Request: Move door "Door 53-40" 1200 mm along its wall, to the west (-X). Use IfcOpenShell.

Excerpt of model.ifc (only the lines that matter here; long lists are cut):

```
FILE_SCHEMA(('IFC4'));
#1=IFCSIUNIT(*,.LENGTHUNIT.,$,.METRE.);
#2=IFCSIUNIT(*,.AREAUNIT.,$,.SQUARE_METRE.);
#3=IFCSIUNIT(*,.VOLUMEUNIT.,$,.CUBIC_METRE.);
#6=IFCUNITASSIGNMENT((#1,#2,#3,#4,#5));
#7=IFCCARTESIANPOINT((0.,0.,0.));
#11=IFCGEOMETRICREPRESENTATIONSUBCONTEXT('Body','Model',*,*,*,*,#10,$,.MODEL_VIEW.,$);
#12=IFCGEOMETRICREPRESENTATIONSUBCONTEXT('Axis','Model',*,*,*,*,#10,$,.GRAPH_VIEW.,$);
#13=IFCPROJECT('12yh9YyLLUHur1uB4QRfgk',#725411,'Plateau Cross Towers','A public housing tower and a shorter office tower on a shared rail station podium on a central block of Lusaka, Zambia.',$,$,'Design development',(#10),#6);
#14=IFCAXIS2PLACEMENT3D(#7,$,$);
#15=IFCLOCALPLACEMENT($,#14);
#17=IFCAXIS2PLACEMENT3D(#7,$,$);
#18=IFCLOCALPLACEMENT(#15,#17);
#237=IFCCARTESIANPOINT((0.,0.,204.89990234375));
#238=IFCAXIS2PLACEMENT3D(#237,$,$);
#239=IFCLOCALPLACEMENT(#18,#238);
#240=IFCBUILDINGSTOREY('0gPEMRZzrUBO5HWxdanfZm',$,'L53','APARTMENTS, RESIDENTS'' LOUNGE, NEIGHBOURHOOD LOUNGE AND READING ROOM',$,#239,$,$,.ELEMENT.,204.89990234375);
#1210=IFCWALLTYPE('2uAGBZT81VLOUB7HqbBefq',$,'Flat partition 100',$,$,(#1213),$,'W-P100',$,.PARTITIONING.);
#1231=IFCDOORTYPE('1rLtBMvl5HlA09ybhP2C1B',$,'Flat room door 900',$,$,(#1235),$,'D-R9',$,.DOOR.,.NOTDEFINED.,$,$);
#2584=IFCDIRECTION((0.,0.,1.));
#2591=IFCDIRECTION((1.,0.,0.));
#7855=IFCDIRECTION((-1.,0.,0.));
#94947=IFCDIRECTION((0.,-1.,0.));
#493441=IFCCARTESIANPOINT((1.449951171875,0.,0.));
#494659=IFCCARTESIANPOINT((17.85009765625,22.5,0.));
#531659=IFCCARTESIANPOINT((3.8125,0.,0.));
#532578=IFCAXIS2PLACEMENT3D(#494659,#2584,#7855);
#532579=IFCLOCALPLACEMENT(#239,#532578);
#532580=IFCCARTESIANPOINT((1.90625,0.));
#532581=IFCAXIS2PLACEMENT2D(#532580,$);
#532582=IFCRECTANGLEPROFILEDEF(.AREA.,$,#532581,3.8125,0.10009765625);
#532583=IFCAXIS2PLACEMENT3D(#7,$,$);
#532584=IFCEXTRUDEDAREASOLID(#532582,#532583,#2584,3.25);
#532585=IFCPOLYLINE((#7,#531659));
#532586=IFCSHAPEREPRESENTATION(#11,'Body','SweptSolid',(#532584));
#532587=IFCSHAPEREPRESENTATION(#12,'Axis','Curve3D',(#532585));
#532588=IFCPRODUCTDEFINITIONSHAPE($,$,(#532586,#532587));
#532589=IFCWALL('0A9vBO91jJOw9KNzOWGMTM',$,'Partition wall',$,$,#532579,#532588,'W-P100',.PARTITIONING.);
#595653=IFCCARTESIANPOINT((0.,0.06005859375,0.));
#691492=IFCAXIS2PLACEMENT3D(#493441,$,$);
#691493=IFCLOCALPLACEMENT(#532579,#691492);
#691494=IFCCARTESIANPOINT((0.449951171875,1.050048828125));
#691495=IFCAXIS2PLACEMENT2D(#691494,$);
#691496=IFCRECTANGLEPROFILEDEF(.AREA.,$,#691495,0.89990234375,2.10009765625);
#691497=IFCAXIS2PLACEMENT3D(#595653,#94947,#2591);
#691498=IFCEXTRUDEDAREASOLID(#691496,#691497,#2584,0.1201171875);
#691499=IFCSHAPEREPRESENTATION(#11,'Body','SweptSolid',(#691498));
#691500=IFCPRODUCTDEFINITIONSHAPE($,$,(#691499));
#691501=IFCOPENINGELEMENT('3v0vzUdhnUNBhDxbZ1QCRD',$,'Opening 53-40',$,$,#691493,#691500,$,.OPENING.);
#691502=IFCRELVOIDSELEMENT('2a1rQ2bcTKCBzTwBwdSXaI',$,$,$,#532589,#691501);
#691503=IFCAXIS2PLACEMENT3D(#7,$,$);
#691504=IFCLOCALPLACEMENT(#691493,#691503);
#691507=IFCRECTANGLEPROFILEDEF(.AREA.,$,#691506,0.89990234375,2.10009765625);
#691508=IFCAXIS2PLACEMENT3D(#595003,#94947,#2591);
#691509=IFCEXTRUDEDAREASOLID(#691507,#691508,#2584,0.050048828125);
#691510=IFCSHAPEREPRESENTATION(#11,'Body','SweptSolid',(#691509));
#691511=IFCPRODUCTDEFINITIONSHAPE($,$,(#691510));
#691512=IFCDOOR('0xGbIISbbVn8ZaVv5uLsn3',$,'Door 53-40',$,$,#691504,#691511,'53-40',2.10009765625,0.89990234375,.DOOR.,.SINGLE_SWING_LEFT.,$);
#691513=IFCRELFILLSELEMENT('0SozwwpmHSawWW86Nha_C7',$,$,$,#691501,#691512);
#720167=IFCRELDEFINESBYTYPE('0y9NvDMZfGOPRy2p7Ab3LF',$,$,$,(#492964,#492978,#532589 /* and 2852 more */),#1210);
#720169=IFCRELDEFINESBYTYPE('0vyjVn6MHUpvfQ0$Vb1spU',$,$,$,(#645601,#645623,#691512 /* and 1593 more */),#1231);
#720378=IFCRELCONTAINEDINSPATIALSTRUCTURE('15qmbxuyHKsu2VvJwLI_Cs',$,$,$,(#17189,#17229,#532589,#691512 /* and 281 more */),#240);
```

```python
import ifcopenshell
import ifcopenshell.api.geometry
import ifcopenshell.util.placement
import ifcopenshell.util.unit

model = ifcopenshell.open("model.ifc")
unit_scale = ifcopenshell.util.unit.calculate_unit_scale(model)

door = model.by_guid("0xGbIISbbVn8ZaVv5uLsn3")
opening = door.FillsVoids[0].RelatingOpeningElement
wall = opening.VoidsElements[0].RelatingBuildingElement

wall_matrix = ifcopenshell.util.placement.get_local_placement(wall.ObjectPlacement)
shift = wall_matrix[:3, 0] * 1.2 / unit_scale
before = ifcopenshell.util.placement.get_local_placement(door.ObjectPlacement)[:3, 3].copy()

# The door is placed relative to its opening, so it follows when the opening moves.
matrix = ifcopenshell.util.placement.get_local_placement(opening.ObjectPlacement)
matrix[:3, 3] += shift
ifcopenshell.api.geometry.edit_object_placement(
    model, product=opening, matrix=matrix, is_si=False, should_transform_children=True
)

after = ifcopenshell.util.placement.get_local_placement(door.ObjectPlacement)[:3, 3]
print("door moved by", (after - before).round(3) + 0.0)

model.write("model_edited.ifc")
```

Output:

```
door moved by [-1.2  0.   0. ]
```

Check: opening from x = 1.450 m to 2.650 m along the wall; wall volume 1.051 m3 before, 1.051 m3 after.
